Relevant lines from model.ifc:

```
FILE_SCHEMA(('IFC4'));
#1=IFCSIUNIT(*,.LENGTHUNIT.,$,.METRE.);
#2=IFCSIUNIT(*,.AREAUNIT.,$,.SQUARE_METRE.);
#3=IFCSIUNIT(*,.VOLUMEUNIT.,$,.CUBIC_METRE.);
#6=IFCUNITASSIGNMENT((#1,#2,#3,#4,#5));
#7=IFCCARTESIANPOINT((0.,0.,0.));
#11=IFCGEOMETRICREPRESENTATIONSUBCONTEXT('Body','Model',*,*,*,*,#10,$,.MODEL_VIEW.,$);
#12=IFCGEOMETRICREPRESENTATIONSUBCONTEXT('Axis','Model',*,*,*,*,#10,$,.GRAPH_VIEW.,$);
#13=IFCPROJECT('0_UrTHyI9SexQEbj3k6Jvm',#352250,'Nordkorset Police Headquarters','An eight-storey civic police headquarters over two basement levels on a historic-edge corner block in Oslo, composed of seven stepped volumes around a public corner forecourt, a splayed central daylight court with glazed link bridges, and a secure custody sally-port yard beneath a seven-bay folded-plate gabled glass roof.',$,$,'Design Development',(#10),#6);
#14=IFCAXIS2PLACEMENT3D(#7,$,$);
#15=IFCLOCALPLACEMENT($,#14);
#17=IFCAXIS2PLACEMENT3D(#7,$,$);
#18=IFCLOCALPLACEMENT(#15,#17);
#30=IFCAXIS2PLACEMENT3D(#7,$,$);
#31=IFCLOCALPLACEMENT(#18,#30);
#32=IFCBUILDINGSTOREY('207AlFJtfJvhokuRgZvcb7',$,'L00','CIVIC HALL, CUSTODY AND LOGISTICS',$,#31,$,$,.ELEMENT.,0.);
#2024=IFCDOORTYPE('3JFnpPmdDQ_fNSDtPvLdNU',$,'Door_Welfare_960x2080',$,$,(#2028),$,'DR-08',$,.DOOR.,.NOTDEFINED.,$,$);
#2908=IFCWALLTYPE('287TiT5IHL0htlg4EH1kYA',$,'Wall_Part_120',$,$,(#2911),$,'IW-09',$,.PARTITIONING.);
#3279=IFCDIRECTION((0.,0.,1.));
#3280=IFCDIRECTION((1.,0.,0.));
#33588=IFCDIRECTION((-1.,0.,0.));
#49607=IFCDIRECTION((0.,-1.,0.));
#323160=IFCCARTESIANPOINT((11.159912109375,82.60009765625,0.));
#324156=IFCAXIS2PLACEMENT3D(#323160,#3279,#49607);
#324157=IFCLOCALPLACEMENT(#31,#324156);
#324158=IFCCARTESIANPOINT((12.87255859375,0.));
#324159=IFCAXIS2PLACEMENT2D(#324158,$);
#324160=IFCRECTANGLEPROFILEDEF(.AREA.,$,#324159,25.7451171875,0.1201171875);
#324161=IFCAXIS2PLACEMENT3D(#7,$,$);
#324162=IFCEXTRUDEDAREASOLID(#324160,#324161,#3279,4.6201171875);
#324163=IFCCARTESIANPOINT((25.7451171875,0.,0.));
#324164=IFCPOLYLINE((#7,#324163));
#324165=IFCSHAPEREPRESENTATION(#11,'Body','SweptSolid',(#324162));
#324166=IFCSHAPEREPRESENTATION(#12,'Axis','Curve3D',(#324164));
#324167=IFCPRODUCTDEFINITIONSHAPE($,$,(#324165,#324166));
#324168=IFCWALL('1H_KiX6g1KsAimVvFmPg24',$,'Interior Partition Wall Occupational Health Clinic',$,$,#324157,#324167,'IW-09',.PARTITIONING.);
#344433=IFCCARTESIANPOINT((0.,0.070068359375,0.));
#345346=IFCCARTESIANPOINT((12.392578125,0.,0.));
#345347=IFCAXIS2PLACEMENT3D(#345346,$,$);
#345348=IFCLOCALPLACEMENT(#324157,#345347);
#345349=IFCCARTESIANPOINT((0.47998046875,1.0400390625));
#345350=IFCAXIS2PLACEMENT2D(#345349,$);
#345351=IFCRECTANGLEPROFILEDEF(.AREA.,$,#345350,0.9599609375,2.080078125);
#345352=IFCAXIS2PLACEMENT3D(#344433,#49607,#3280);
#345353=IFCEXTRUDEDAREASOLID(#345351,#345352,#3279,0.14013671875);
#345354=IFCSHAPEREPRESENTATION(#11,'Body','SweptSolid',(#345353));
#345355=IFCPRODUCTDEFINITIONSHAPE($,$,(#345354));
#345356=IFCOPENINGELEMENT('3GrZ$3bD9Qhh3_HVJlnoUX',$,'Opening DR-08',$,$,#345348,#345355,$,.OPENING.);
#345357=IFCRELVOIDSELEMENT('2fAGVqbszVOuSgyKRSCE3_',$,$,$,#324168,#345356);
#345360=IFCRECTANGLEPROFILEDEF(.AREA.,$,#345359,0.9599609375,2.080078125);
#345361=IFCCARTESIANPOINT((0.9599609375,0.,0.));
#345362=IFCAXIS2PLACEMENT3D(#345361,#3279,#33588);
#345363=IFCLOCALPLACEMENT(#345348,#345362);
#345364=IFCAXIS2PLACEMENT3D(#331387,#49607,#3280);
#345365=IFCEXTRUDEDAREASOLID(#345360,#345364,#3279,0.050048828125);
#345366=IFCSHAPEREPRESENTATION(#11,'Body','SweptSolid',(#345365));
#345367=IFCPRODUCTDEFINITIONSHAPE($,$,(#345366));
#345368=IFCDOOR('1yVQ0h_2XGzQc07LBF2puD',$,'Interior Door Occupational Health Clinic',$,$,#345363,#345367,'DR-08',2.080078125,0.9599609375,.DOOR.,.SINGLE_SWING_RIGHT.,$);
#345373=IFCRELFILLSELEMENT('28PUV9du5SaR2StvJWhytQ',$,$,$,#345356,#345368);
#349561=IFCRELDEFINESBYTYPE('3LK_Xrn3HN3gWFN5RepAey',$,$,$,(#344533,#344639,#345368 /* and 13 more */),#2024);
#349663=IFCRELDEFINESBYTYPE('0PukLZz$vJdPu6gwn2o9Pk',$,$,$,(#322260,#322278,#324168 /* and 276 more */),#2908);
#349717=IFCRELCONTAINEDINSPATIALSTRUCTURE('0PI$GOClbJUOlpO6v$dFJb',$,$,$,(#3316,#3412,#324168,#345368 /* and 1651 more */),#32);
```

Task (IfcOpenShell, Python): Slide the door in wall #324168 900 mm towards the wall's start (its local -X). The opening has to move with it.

```python
import ifcopenshell
import ifcopenshell.api.geometry
import ifcopenshell.util.placement
import ifcopenshell.util.unit

model = ifcopenshell.open("model.ifc")
unit_scale = ifcopenshell.util.unit.calculate_unit_scale(model)

door = model.by_guid("1yVQ0h_2XGzQc07LBF2puD")
opening = door.FillsVoids[0].RelatingOpeningElement
wall = opening.VoidsElements[0].RelatingBuildingElement

wall_matrix = ifcopenshell.util.placement.get_local_placement(wall.ObjectPlacement)
shift = wall_matrix[:3, 0] * -0.9 / unit_scale
before = ifcopenshell.util.placement.get_local_placement(door.ObjectPlacement)[:3, 3].copy()

# The door is placed relative to its opening, so it follows when the opening moves.
matrix = ifcopenshell.util.placement.get_local_placement(opening.ObjectPlacement)
matrix[:3, 3] += shift
ifcopenshell.api.geometry.edit_object_placement(
    model, product=opening, matrix=matrix, is_si=False, should_transform_children=True
)

after = ifcopenshell.util.placement.get_local_placement(door.ObjectPlacement)[:3, 3]
print("door moved by", (after - before).round(3) + 0.0)

model.write("model-out.ifc")
```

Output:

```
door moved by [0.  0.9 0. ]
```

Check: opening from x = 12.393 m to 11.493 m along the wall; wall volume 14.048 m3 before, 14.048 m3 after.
